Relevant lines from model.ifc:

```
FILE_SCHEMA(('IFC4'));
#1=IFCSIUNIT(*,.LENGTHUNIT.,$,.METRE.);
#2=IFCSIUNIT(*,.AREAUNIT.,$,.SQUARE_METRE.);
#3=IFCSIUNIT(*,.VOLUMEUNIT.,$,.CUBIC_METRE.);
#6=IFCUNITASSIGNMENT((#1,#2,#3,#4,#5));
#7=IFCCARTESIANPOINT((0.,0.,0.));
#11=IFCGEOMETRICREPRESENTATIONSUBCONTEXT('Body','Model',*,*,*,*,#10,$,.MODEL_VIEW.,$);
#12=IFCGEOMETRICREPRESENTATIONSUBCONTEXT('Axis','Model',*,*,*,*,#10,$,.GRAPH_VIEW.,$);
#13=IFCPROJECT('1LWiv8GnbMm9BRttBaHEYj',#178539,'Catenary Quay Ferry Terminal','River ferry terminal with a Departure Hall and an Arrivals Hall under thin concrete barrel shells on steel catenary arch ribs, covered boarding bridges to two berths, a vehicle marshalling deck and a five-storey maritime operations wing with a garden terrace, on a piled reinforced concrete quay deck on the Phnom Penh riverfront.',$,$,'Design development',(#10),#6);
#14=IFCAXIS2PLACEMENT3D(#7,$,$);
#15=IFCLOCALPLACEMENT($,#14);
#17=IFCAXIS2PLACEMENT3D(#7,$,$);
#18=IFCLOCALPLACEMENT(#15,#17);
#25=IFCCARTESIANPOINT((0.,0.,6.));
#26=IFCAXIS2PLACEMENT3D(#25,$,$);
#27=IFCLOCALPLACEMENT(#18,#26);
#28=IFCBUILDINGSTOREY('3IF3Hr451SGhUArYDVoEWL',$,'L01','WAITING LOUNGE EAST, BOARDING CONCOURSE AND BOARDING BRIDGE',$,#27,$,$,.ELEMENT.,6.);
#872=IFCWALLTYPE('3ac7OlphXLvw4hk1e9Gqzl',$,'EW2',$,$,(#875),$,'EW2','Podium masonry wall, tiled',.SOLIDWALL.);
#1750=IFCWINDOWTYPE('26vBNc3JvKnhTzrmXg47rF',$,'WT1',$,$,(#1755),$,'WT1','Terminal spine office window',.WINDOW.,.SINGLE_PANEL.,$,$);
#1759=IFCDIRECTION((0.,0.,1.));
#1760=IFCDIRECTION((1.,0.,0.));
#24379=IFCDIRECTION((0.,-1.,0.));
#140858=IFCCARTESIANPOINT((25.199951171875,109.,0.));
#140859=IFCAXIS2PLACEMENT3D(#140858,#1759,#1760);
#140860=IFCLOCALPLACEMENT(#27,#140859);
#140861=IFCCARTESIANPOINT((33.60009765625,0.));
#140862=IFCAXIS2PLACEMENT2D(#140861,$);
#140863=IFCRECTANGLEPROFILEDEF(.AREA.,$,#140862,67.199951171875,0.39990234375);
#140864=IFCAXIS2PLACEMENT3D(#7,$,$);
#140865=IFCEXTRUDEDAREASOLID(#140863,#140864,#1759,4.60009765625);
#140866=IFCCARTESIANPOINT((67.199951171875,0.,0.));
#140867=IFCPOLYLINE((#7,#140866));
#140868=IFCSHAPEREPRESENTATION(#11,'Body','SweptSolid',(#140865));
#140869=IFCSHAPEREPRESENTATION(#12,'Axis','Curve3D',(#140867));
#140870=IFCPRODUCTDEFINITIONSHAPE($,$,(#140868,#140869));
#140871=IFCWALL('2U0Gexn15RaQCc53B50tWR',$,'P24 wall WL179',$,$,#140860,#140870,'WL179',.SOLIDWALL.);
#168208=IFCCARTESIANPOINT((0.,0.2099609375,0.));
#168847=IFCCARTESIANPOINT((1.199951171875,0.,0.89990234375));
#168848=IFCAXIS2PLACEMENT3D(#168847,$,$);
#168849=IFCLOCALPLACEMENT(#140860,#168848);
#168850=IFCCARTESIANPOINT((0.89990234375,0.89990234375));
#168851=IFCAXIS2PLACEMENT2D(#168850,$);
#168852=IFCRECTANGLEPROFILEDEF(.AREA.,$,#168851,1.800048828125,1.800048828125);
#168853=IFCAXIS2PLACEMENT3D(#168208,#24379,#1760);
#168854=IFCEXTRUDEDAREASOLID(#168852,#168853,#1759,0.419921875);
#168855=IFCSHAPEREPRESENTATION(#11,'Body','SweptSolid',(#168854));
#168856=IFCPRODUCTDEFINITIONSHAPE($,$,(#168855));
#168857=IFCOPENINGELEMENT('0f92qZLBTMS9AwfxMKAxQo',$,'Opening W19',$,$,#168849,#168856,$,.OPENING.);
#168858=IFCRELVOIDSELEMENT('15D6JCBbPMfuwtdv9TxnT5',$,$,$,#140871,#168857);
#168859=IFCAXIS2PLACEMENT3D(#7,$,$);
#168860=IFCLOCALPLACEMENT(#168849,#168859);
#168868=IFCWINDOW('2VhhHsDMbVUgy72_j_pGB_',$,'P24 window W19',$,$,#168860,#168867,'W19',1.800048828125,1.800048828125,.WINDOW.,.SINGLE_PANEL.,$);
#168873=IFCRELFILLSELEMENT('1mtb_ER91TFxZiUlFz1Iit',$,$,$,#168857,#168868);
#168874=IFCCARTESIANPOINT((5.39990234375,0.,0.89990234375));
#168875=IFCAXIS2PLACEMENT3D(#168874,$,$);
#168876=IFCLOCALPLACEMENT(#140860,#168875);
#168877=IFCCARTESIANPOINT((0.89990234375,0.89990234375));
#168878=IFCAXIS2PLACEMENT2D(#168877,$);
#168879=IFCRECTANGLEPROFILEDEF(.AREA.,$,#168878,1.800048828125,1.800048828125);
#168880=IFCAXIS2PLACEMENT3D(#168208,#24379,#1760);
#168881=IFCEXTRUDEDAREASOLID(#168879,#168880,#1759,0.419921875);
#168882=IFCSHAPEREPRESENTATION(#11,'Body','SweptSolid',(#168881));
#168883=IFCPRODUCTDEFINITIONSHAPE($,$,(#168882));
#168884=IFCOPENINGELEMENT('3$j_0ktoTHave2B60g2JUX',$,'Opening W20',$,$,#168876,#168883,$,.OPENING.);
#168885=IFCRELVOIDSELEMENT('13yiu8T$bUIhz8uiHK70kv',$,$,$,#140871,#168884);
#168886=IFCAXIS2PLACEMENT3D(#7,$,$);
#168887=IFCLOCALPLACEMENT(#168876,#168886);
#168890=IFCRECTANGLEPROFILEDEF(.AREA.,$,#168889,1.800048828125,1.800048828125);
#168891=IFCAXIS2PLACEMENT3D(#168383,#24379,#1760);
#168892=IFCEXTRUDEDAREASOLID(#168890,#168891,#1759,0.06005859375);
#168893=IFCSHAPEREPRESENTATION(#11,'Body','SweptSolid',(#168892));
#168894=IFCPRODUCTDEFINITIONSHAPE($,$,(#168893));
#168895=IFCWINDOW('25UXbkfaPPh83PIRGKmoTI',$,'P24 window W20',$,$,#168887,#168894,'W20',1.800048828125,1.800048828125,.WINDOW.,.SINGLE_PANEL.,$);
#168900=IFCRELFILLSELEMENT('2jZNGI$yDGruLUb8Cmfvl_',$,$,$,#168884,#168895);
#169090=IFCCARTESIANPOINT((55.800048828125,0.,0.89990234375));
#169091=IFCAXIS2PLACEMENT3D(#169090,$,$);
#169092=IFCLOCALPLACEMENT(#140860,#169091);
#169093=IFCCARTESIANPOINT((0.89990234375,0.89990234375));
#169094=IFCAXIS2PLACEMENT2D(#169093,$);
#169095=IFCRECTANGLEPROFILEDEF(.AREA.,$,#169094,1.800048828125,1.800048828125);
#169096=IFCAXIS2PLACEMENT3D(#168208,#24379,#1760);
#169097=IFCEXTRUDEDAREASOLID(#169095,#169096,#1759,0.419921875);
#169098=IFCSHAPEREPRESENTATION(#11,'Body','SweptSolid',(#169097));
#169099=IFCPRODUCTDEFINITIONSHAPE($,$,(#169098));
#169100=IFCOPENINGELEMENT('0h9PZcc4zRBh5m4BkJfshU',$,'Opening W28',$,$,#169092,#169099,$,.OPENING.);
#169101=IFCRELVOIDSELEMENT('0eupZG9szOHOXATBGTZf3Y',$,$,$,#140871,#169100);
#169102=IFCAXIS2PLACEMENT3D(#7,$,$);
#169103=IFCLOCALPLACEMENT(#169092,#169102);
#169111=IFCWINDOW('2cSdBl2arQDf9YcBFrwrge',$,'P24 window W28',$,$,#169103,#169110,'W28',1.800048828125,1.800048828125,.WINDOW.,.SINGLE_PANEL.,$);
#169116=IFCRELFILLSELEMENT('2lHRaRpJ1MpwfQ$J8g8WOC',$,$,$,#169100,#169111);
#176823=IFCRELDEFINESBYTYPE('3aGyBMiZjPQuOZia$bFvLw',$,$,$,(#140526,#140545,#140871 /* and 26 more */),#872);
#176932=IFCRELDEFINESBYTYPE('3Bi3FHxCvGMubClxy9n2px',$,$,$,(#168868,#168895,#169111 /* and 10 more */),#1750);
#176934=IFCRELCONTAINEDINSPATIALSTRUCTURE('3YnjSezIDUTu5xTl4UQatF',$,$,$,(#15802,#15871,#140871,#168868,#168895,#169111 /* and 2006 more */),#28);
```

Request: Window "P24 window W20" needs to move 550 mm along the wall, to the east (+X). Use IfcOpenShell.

```python
import ifcopenshell
import ifcopenshell.api.geometry
import ifcopenshell.util.placement

model = ifcopenshell.open("model.ifc")

window = model.by_guid("25UXbkfaPPh83PIRGKmoTI")
opening = window.FillsVoids[0].RelatingOpeningElement
wall = opening.VoidsElements[0].RelatingBuildingElement

wall_matrix = ifcopenshell.util.placement.get_local_placement(wall.ObjectPlacement)
shift = wall_matrix[:3, 0] * 0.55
before = ifcopenshell.util.placement.get_local_placement(window.ObjectPlacement)[:3, 3].copy()

# The window is placed relative to its opening, so it follows when the opening moves.
matrix = ifcopenshell.util.placement.get_local_placement(opening.ObjectPlacement)
matrix[:3, 3] += shift
ifcopenshell.api.geometry.edit_object_placement(
    model, product=opening, matrix=matrix, is_si=False, should_transform_children=True
)

after = ifcopenshell.util.placement.get_local_placement(window.ObjectPlacement)[:3, 3]
print("window moved by", (after - before).round(3) + 0.0)

model.write("model_v2.ifc")
```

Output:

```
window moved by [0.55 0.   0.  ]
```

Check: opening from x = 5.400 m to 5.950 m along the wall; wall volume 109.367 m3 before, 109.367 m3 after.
